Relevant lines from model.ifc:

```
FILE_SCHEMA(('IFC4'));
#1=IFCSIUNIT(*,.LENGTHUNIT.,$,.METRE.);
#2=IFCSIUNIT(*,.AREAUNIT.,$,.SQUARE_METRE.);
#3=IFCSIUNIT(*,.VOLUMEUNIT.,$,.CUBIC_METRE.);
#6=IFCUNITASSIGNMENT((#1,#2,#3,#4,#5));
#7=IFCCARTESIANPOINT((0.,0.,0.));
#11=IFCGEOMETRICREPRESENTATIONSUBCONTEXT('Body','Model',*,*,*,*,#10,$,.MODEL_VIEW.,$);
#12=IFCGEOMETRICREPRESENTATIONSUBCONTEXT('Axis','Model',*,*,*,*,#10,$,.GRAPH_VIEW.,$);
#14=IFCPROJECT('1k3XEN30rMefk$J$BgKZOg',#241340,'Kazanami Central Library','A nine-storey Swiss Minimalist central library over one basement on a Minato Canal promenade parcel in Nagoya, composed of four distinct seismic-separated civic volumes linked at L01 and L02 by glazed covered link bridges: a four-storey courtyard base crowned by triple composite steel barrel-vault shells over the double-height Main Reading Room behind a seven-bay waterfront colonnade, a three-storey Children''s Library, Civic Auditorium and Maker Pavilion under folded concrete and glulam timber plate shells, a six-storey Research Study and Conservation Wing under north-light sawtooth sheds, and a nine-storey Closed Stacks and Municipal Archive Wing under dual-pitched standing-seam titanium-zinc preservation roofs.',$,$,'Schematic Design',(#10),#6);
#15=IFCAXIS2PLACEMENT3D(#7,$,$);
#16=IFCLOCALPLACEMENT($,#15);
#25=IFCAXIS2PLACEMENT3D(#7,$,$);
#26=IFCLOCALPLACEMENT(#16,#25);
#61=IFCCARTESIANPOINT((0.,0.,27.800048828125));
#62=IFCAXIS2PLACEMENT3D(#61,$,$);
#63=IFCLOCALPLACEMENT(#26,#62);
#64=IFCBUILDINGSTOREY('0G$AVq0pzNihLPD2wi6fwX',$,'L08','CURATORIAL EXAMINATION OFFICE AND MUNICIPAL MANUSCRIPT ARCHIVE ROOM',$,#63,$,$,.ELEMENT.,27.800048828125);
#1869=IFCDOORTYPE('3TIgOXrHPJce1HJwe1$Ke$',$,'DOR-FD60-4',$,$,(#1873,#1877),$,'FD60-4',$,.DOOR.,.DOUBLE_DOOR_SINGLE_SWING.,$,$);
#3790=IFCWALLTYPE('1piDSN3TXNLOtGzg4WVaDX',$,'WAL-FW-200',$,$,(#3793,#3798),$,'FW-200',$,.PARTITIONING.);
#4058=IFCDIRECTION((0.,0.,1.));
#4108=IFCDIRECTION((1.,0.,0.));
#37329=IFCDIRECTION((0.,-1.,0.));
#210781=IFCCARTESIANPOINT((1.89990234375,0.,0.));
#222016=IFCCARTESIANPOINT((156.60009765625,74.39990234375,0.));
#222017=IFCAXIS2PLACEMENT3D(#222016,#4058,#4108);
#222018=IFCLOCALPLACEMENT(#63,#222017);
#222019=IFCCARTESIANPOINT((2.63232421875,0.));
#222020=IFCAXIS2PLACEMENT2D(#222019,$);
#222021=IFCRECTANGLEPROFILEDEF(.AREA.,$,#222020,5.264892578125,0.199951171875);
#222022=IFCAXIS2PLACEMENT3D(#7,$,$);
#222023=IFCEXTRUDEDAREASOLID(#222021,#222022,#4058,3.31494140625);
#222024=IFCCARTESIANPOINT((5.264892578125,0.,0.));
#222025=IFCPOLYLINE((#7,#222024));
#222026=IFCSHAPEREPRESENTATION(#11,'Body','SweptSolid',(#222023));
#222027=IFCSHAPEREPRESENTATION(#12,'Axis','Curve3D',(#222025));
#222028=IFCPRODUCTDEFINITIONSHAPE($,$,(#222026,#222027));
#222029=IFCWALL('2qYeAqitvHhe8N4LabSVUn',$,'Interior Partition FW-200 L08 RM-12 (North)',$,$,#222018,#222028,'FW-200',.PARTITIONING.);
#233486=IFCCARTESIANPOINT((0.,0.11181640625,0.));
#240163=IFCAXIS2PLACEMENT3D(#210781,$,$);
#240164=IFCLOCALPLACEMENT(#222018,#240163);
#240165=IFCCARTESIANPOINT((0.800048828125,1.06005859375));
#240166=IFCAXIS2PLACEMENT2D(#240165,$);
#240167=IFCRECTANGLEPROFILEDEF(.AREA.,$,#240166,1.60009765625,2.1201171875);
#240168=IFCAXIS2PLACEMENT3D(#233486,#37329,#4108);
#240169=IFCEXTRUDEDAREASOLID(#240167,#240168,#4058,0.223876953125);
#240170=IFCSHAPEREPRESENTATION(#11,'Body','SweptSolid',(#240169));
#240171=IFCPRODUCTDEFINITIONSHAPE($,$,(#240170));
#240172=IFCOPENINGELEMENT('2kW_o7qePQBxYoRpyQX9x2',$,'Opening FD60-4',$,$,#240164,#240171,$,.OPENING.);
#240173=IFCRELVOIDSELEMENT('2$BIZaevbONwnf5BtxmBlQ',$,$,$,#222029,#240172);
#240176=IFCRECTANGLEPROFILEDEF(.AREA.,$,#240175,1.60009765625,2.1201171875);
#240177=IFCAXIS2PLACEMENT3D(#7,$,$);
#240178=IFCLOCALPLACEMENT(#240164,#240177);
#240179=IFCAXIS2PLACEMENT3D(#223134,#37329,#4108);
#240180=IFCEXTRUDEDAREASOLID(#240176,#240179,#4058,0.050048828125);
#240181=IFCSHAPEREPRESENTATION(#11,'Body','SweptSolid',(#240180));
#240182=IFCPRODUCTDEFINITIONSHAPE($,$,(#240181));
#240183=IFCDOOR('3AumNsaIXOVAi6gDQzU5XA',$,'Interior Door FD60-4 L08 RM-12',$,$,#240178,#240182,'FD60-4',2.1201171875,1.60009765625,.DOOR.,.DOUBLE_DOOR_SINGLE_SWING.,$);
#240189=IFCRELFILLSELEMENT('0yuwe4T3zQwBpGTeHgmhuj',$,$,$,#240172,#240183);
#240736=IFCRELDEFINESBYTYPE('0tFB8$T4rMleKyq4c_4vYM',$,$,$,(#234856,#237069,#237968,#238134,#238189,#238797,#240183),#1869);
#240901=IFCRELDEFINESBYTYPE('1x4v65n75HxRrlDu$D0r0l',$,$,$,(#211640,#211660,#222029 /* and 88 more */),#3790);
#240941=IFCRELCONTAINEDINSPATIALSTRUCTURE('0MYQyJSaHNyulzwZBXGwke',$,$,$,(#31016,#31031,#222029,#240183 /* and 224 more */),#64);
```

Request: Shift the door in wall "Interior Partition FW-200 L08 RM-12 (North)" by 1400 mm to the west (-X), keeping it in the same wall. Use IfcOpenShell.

```python
import ifcopenshell
import ifcopenshell.api.geometry
import ifcopenshell.util.placement
import ifcopenshell.util.unit

model = ifcopenshell.open("model.ifc")
unit_scale = ifcopenshell.util.unit.calculate_unit_scale(model)

door = model.by_guid("3AumNsaIXOVAi6gDQzU5XA")
opening = door.FillsVoids[0].RelatingOpeningElement
wall = opening.VoidsElements[0].RelatingBuildingElement

wall_matrix = ifcopenshell.util.placement.get_local_placement(wall.ObjectPlacement)
shift = wall_matrix[:3, 0] * -1.4 / unit_scale
before = ifcopenshell.util.placement.get_local_placement(door.ObjectPlacement)[:3, 3].copy()

# The door is placed relative to its opening, so it follows when the opening moves.
matrix = ifcopenshell.util.placement.get_local_placement(opening.ObjectPlacement)
matrix[:3, 3] += shift
ifcopenshell.api.geometry.edit_object_placement(
    model, product=opening, matrix=matrix, is_si=False, should_transform_children=True
)

after = ifcopenshell.util.placement.get_local_placement(door.ObjectPlacement)[:3, 3]
print("door moved by", (after - before).round(3) + 0.0)

model.write("model_updated.ifc")
```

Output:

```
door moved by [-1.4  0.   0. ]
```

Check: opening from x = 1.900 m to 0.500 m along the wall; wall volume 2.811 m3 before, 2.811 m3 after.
